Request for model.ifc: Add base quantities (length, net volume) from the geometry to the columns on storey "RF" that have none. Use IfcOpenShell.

First a look at what the model holds.

```python
import ifcopenshell
import ifcopenshell.util.element
import ifcopenshell.util.unit

model = ifcopenshell.open("model.ifc")
print(model.schema)
for unit_type in ("LENGTHUNIT", "AREAUNIT", "VOLUMEUNIT"):
    print(unit_type, ifcopenshell.util.unit.calculate_unit_scale(model, unit_type))
storey = next(s for s in model.by_type("IfcBuildingStorey") if s.Name == "RF")
columns = [e for e in ifcopenshell.util.element.get_decomposition(storey) if e.is_a("IfcColumn")]
for e in sorted(columns, key=lambda e: e.id()):
    print(e.id(), e.is_a(), e.Name, list(ifcopenshell.util.element.get_psets(e, qtos_only=True)), sep=" | ")
```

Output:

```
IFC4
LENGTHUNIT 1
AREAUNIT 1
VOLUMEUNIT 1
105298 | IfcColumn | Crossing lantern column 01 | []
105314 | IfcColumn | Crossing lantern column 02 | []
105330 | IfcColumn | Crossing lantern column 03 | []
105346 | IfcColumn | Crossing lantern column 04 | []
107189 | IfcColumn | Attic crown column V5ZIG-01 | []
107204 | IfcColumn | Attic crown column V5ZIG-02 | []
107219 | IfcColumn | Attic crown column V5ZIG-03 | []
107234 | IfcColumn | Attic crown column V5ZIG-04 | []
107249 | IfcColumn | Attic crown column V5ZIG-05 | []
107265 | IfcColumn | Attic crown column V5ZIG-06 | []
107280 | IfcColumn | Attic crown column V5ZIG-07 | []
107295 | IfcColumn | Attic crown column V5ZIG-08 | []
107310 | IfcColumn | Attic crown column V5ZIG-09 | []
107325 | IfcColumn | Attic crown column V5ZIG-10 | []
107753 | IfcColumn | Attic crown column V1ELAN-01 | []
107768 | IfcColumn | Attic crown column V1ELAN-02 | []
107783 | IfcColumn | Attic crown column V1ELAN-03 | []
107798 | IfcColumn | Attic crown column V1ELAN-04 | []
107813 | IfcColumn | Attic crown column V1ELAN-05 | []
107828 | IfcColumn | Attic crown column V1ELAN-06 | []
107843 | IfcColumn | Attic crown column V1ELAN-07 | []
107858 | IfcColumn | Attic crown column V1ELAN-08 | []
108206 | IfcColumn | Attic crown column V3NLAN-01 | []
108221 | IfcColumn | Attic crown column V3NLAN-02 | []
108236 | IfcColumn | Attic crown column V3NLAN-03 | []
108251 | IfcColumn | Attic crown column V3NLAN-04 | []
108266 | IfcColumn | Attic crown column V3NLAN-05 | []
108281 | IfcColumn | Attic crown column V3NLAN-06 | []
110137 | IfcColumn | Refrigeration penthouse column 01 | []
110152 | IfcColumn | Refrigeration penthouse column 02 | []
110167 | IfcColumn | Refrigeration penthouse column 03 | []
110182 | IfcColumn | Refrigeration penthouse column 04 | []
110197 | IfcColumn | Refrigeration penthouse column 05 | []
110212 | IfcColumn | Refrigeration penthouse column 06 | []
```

```python
import ifcopenshell
import ifcopenshell.api.pset
import ifcopenshell.geom
import ifcopenshell.util.element
import ifcopenshell.util.shape
import ifcopenshell.util.unit

model = ifcopenshell.open("model.ifc")
unit_scale = ifcopenshell.util.unit.calculate_unit_scale(model)
volume_scale = ifcopenshell.util.unit.calculate_unit_scale(model, "VOLUMEUNIT")
settings = ifcopenshell.geom.settings()

storey = next(s for s in model.by_type("IfcBuildingStorey") if s.Name == "RF")
columns = [e for e in ifcopenshell.util.element.get_decomposition(storey) if e.is_a("IfcColumn")]

for e in sorted(columns, key=lambda e: e.id()):
    if ifcopenshell.util.element.get_psets(e, qtos_only=True, should_inherit=False):
        continue
    # Geometry comes back in metres, in the element's own axes.
    shape = ifcopenshell.geom.create_shape(settings, e)
    values = {
        "Length": ifcopenshell.util.shape.get_z(shape.geometry) / unit_scale,
        "NetVolume": ifcopenshell.util.shape.get_volume(shape.geometry) / volume_scale,
    }
    qto = ifcopenshell.api.pset.add_qto(model, product=e, name="Qto_ColumnBaseQuantities")
    ifcopenshell.api.pset.edit_qto(model, qto=qto, properties=values)
    print(e.id(), {k: round(v, 3) for k, v in values.items()})

model.write("model_v2.ifc")
```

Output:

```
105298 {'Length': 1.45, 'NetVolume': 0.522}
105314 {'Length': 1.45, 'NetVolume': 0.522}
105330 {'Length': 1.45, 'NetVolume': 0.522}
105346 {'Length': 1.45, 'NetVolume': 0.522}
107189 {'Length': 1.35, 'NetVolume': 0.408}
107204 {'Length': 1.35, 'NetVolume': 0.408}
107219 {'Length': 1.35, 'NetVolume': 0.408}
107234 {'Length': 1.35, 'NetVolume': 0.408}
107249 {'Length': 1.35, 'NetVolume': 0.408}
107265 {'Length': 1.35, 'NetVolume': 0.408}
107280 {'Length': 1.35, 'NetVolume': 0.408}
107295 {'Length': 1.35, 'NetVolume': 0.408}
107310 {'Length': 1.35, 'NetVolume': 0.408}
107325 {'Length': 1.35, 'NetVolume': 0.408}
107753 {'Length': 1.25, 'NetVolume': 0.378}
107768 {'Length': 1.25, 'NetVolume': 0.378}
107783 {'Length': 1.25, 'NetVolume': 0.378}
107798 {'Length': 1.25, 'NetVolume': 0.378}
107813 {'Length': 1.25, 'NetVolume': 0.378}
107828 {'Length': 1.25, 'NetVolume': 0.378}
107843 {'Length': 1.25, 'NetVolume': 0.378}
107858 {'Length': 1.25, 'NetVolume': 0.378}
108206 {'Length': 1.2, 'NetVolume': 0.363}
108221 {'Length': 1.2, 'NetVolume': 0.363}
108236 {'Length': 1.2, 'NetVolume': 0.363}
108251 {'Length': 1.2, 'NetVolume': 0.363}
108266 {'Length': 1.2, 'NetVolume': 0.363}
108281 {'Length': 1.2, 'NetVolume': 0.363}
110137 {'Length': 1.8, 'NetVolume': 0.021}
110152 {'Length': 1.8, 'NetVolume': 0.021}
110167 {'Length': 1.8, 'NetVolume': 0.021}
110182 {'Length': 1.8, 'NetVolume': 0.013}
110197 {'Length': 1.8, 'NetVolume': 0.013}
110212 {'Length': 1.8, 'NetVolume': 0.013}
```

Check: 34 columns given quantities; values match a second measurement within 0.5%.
